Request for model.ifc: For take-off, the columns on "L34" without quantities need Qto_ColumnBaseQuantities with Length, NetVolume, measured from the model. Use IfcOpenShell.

First a look at what the model holds.

```python
import ifcopenshell
import ifcopenshell.util.element
import ifcopenshell.util.unit

model = ifcopenshell.open("model.ifc")
print(model.schema)
for unit_type in ("LENGTHUNIT", "AREAUNIT", "VOLUMEUNIT"):
    print(unit_type, ifcopenshell.util.unit.calculate_unit_scale(model, unit_type))
storey = next(s for s in model.by_type("IfcBuildingStorey") if s.Name == "L34")
columns = [e for e in ifcopenshell.util.element.get_decomposition(storey) if e.is_a("IfcColumn")]
for e in sorted(columns, key=lambda e: e.id()):
    print(e.id(), e.is_a(), e.Name, list(ifcopenshell.util.element.get_psets(e, qtos_only=True)), sep=" | ")
```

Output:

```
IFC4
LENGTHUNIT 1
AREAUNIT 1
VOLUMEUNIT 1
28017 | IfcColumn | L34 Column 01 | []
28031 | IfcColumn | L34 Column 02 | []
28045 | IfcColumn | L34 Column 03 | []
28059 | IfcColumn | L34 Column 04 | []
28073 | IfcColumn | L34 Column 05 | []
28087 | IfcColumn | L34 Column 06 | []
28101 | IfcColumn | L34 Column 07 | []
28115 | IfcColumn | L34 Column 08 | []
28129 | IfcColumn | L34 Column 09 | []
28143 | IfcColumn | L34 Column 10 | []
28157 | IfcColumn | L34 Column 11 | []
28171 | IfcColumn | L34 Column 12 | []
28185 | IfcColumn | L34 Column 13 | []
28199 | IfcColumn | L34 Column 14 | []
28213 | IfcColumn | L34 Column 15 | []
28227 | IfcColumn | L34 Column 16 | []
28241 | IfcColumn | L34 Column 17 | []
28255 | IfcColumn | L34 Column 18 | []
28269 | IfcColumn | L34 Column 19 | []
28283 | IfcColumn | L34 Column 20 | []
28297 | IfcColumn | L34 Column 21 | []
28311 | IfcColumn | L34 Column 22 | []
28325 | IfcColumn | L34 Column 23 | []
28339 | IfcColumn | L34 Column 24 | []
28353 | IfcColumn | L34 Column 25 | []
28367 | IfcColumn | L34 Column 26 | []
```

```python
import ifcopenshell
import ifcopenshell.api.pset
import ifcopenshell.geom
import ifcopenshell.util.element
import ifcopenshell.util.shape
import ifcopenshell.util.unit

model = ifcopenshell.open("model.ifc")
unit_scale = ifcopenshell.util.unit.calculate_unit_scale(model)
volume_scale = ifcopenshell.util.unit.calculate_unit_scale(model, "VOLUMEUNIT")
settings = ifcopenshell.geom.settings()

storey = next(s for s in model.by_type("IfcBuildingStorey") if s.Name == "L34")
columns = [e for e in ifcopenshell.util.element.get_decomposition(storey) if e.is_a("IfcColumn")]

for e in sorted(columns, key=lambda e: e.id()):
    if ifcopenshell.util.element.get_psets(e, qtos_only=True, should_inherit=False):
        continue
    # Geometry comes back in metres, in the element's own axes.
    shape = ifcopenshell.geom.create_shape(settings, e)
    values = {
        "Length": ifcopenshell.util.shape.get_z(shape.geometry) / unit_scale,
        "NetVolume": ifcopenshell.util.shape.get_volume(shape.geometry) / volume_scale,
    }
    qto = ifcopenshell.api.pset.add_qto(model, product=e, name="Qto_ColumnBaseQuantities")
    ifcopenshell.api.pset.edit_qto(model, qto=qto, properties=values)
    print(e.id(), {k: round(v, 3) for k, v in values.items()})

model.write("model_v2.ifc")
```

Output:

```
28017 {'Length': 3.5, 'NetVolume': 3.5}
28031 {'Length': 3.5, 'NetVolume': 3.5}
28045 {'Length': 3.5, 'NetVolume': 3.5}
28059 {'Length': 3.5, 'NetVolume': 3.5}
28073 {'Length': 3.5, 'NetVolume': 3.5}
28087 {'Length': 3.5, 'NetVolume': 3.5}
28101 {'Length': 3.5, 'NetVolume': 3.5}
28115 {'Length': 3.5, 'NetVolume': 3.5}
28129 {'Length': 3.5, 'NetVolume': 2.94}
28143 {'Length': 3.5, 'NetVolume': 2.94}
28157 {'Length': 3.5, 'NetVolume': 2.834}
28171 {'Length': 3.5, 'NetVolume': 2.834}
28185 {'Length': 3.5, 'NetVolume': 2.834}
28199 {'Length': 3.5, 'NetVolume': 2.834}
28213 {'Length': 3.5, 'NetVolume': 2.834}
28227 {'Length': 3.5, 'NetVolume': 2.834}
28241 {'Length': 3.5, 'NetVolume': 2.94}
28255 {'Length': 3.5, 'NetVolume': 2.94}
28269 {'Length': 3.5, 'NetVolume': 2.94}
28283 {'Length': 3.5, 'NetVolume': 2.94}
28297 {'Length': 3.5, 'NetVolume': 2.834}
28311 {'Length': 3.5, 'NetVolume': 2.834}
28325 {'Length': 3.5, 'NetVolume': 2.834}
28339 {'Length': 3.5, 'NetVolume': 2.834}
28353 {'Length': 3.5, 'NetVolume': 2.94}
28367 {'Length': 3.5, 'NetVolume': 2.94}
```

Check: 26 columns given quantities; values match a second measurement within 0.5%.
